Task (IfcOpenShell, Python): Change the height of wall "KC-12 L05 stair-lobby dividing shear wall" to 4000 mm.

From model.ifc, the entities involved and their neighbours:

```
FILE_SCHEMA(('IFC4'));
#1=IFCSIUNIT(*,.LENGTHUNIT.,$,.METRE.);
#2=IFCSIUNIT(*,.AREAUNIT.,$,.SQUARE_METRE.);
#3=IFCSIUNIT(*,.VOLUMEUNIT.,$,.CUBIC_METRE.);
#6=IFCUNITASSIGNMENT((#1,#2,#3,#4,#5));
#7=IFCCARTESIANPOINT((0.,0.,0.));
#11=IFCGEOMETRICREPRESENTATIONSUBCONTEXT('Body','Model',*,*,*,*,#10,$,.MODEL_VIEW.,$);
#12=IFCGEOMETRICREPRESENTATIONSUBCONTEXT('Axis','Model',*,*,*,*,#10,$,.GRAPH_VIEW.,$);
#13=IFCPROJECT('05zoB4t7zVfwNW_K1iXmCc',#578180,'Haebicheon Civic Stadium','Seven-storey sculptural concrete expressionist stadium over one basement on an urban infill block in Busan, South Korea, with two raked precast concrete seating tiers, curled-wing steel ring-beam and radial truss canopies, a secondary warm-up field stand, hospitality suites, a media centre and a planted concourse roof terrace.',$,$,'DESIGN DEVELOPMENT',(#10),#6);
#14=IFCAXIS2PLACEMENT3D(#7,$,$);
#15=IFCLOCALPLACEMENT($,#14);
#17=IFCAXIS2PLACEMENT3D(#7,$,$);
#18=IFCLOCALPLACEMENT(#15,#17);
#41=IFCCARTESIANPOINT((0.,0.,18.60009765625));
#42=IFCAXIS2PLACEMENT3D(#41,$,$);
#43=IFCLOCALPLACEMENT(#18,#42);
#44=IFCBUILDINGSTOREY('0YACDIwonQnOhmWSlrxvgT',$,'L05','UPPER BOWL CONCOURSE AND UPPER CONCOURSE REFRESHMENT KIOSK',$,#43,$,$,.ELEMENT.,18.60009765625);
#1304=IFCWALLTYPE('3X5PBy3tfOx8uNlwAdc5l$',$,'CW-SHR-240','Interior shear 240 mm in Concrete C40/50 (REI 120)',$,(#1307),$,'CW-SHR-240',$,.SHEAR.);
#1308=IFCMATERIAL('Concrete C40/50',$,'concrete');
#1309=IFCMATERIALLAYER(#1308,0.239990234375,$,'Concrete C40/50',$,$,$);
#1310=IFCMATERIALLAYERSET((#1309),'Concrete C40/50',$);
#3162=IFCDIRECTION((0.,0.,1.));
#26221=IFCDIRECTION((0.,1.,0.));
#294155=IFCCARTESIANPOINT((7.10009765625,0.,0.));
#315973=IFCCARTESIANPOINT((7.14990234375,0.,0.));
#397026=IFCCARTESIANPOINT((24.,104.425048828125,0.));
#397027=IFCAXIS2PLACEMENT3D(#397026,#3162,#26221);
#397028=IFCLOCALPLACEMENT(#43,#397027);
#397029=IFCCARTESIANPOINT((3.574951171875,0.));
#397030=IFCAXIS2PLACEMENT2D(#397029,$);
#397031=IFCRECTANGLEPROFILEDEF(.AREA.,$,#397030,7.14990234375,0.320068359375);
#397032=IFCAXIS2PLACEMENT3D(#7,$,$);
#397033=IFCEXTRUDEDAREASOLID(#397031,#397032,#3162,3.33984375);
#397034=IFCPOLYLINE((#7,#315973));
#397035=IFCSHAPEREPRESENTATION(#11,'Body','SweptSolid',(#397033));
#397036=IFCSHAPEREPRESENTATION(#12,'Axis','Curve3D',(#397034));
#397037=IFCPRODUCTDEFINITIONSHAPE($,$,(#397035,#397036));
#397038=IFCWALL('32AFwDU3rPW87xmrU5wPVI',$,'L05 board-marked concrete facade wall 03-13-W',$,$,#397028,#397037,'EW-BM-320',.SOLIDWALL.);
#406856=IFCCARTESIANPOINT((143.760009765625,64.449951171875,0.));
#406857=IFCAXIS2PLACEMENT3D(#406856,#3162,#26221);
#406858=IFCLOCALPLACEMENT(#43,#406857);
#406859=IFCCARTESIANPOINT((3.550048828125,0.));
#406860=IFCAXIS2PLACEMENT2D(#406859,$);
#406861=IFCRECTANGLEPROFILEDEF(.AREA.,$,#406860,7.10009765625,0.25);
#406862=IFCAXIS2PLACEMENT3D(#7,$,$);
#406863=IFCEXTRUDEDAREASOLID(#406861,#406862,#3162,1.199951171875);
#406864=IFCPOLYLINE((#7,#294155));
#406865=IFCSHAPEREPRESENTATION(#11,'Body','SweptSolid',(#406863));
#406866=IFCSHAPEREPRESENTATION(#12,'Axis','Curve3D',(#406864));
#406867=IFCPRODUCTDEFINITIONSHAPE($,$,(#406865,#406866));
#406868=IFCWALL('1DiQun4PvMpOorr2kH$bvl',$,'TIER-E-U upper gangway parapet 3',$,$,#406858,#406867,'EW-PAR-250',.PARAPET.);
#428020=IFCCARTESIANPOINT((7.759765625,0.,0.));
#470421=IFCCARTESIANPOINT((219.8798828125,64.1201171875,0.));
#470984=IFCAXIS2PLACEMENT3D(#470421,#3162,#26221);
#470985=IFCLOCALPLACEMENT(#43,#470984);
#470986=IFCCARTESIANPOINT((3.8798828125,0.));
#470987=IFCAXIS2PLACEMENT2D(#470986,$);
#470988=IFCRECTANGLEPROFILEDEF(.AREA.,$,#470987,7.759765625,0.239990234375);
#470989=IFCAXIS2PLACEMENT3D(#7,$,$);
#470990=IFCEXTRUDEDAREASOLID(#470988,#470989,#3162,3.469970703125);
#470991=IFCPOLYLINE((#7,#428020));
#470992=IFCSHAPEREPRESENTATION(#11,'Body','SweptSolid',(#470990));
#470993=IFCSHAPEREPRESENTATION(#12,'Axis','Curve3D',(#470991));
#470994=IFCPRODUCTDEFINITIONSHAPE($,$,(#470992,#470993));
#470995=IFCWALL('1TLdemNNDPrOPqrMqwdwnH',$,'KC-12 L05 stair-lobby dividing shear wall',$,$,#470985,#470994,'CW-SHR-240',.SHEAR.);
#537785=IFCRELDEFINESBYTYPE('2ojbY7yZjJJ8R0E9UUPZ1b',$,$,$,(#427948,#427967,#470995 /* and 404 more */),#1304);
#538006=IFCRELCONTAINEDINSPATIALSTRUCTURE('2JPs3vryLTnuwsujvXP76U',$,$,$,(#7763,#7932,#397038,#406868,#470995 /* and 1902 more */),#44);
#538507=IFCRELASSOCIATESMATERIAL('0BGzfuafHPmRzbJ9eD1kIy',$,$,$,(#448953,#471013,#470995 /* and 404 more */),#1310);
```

```python
import ifcopenshell
import ifcopenshell.geom
import ifcopenshell.util.representation
import ifcopenshell.util.shape
import ifcopenshell.util.unit

model = ifcopenshell.open("model.ifc")
unit_scale = ifcopenshell.util.unit.calculate_unit_scale(model)
settings = ifcopenshell.geom.settings()


def volume(element):
    """Net volume in cubic metres, openings subtracted."""
    shape = ifcopenshell.geom.create_shape(settings, element)
    return ifcopenshell.util.shape.get_volume(shape.geometry)


wall = model.by_guid("1TLdemNNDPrOPqrMqwdwnH")
before = volume(wall)

body = ifcopenshell.util.representation.get_representation(wall, "Model", "Body")
solid = body.Items[0]
old_height = solid.Depth
solid.Depth = 4 / unit_scale
after = volume(wall)

print(f"height {old_height:g} -> {solid.Depth:g}, volume {before:.3f} -> {after:.3f} m3")

model.write("model_edited.ifc")
```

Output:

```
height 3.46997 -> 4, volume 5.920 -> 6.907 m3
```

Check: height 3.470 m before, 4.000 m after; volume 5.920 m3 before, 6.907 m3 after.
